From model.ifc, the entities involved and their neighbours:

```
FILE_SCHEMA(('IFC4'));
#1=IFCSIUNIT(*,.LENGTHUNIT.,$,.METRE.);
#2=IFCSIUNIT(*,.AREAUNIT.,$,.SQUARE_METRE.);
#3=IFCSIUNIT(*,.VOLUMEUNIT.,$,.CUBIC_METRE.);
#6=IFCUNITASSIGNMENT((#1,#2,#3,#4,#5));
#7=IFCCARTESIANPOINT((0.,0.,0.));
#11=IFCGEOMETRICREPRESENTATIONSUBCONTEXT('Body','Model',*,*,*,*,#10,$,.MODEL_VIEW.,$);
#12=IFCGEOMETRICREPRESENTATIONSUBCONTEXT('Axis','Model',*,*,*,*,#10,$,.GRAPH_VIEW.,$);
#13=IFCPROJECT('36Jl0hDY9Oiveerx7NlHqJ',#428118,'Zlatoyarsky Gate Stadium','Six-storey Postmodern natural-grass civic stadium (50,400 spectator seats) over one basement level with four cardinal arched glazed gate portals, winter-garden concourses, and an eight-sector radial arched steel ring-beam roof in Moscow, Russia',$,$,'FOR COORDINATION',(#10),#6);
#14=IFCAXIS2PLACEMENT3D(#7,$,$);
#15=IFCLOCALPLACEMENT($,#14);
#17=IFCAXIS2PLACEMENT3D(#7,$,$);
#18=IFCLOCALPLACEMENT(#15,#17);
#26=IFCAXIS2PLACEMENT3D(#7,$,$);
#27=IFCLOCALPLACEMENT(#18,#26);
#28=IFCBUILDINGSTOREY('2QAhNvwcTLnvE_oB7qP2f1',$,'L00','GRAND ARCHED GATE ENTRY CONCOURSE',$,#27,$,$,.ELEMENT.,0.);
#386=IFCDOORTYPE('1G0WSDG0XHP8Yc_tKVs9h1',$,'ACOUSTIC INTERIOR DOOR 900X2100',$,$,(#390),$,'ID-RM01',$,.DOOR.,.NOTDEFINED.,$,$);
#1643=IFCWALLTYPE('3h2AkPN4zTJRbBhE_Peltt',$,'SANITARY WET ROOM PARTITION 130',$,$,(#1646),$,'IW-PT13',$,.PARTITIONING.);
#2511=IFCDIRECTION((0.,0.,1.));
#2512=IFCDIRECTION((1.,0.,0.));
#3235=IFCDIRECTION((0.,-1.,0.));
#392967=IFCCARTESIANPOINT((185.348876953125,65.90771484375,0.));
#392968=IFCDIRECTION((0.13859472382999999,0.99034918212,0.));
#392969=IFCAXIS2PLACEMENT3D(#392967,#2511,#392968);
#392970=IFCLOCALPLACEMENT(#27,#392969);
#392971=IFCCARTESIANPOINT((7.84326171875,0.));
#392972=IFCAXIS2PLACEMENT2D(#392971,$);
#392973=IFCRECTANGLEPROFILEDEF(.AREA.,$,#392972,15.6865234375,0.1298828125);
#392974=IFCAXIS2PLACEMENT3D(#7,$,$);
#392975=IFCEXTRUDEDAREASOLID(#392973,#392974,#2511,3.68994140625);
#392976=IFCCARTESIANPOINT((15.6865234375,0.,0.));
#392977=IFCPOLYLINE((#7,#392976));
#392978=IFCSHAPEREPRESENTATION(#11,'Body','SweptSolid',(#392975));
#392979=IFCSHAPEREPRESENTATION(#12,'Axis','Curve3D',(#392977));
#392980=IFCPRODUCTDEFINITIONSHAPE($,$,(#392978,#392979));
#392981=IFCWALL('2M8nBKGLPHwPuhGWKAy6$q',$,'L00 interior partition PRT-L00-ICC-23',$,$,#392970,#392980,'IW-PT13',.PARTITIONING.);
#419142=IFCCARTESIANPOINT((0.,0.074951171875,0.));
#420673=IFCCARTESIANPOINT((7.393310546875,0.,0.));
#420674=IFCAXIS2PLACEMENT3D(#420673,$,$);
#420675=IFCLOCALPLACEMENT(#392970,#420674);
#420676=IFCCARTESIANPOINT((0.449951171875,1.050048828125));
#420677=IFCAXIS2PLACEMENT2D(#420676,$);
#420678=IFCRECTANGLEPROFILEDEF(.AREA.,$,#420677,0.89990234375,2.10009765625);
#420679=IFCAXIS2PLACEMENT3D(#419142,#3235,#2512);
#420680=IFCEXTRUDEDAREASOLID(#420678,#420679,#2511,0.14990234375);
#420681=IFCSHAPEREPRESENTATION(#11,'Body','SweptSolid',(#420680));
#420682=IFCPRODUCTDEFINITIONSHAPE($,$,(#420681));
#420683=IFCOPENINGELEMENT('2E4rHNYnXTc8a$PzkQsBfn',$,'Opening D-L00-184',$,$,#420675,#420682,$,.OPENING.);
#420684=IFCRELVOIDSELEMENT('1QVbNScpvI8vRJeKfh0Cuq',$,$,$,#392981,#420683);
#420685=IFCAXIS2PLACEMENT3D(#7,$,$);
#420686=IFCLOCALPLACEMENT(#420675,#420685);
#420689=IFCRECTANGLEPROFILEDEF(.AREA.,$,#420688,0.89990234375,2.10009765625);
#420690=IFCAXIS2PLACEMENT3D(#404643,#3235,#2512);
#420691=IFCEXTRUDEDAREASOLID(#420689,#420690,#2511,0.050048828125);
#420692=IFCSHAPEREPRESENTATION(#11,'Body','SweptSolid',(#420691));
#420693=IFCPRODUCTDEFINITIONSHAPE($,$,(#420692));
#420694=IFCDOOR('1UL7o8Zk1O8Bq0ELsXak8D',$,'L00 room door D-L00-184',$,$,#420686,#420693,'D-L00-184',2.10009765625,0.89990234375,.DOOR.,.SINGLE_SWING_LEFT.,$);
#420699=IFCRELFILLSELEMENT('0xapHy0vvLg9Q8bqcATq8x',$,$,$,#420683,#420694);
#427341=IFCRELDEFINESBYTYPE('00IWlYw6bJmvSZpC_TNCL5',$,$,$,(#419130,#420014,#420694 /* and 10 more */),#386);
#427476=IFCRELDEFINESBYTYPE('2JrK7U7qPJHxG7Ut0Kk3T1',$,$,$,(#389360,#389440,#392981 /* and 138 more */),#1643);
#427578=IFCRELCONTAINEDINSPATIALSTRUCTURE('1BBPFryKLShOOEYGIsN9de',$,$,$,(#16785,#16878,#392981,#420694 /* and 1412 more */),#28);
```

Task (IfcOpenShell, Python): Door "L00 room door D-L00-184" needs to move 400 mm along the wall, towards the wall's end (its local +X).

```python
import ifcopenshell
import ifcopenshell.api.geometry
import ifcopenshell.util.placement

model = ifcopenshell.open("model.ifc")

door = model.by_guid("1UL7o8Zk1O8Bq0ELsXak8D")
opening = door.FillsVoids[0].RelatingOpeningElement
wall = opening.VoidsElements[0].RelatingBuildingElement

wall_matrix = ifcopenshell.util.placement.get_local_placement(wall.ObjectPlacement)
shift = wall_matrix[:3, 0] * 0.4
before = ifcopenshell.util.placement.get_local_placement(door.ObjectPlacement)[:3, 3].copy()

# The door is placed relative to its opening, so it follows when the opening moves.
matrix = ifcopenshell.util.placement.get_local_placement(opening.ObjectPlacement)
matrix[:3, 3] += shift
ifcopenshell.api.geometry.edit_object_placement(
    model, product=opening, matrix=matrix, is_si=False, should_transform_children=True
)

after = ifcopenshell.util.placement.get_local_placement(door.ObjectPlacement)[:3, 3]
print("door moved by", (after - before).round(3) + 0.0)

model.write("model_rev.ifc")
```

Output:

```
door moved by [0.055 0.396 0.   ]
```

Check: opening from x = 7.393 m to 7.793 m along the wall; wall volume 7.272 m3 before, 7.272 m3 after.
